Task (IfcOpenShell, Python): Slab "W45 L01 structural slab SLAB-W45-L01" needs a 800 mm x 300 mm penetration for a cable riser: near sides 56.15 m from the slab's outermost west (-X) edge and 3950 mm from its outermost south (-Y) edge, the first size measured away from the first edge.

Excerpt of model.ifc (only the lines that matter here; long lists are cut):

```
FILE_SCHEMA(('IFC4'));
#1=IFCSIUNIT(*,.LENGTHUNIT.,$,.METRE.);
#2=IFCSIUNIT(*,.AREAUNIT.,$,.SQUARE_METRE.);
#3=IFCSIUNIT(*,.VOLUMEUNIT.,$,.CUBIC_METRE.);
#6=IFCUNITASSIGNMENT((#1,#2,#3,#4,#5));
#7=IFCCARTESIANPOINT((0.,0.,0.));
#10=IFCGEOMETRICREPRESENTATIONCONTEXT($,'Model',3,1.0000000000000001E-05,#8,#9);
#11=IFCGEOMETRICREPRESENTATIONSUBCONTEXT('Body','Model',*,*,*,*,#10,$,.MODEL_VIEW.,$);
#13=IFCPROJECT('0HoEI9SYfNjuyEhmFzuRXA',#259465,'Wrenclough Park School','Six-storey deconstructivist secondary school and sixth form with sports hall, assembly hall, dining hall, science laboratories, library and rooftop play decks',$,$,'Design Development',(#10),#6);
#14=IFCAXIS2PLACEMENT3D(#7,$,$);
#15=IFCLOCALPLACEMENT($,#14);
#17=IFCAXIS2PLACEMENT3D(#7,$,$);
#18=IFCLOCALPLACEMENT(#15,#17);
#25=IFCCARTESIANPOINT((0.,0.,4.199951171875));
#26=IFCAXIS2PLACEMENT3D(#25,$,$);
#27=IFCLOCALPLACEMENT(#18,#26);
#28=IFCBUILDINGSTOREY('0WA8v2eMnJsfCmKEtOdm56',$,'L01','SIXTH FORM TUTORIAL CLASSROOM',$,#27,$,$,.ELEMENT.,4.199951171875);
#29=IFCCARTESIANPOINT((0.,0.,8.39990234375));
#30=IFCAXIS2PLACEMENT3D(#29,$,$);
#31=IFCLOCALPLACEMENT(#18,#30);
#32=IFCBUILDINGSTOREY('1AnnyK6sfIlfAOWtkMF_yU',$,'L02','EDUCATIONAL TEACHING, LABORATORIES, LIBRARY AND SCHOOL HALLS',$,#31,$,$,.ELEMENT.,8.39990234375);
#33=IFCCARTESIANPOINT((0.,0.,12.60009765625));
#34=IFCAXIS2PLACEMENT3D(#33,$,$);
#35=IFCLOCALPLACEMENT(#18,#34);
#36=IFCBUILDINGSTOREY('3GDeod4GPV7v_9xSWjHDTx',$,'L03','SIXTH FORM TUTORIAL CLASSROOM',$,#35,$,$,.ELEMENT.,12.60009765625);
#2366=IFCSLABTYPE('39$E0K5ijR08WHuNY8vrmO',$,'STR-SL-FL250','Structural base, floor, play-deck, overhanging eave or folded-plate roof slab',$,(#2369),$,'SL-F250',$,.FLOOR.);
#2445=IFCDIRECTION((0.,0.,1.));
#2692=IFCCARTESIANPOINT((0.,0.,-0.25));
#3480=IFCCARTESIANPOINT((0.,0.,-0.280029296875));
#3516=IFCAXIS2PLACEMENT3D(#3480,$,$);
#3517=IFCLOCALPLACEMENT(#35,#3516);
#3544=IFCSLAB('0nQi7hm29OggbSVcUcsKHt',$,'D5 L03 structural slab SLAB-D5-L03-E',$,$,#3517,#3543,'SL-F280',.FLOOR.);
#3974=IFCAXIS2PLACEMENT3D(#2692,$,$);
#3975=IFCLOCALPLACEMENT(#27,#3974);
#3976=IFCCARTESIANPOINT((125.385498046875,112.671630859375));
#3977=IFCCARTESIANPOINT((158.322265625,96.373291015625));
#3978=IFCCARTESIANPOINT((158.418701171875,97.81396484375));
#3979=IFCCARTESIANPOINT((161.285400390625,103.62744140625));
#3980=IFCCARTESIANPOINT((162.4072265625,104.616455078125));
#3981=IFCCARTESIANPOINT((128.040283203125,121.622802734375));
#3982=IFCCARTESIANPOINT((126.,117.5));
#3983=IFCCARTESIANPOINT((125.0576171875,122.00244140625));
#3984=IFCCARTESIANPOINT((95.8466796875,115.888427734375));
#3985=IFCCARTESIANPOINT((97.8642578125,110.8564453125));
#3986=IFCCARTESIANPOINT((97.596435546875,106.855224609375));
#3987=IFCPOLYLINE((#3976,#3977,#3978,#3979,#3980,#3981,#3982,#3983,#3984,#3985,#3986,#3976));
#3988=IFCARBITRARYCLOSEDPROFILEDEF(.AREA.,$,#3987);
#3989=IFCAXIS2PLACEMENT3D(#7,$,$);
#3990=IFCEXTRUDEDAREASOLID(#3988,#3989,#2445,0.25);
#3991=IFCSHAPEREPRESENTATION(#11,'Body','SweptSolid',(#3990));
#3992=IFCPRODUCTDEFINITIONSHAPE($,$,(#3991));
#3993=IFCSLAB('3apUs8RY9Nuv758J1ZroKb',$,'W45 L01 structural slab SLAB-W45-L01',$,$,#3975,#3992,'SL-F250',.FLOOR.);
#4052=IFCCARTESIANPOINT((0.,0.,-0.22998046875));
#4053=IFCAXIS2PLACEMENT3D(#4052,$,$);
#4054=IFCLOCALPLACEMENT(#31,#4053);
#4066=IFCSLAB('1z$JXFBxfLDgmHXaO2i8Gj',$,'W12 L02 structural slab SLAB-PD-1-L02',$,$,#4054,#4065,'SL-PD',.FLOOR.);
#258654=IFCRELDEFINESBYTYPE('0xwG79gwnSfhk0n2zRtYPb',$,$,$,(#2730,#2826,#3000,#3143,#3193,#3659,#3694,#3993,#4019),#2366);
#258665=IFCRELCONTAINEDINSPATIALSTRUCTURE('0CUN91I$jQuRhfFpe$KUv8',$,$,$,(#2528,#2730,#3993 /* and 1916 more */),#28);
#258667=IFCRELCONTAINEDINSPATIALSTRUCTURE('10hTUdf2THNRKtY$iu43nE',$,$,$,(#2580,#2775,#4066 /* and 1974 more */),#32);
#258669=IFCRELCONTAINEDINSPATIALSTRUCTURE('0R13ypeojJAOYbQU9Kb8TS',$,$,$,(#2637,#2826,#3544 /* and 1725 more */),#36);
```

```python
import numpy as np
import ifcopenshell
import ifcopenshell.api.feature
import ifcopenshell.api.geometry
import ifcopenshell.api.root
import ifcopenshell.geom
import ifcopenshell.util.placement
import ifcopenshell.util.representation
import ifcopenshell.util.shape
import ifcopenshell.util.unit

model = ifcopenshell.open("model.ifc")
unit_scale = ifcopenshell.util.unit.calculate_unit_scale(model)
settings = ifcopenshell.geom.settings()


def volume(element):
    """Net volume in cubic metres, openings subtracted."""
    shape = ifcopenshell.geom.create_shape(settings, element)
    return ifcopenshell.util.shape.get_volume(shape.geometry)


slab = model.by_guid("3apUs8RY9Nuv758J1ZroKb")
before = volume(slab)

# Extent in the slab's own axes, in metres. The edges named are its -X and -Y sides.
slab_shape = ifcopenshell.geom.create_shape(settings, slab)
vertices = ifcopenshell.util.shape.get_vertices(slab_shape.geometry)
x_min, y_min, bottom = vertices.min(axis=0)
top = vertices[:, 2].max()

opening = ifcopenshell.api.root.create_entity(model, ifc_class="IfcOpeningElement", name="Cable riser opening", predefined_type="OPENING")
context = ifcopenshell.util.representation.get_context(model, "Model", "Body", "MODEL_VIEW")
width, depth = 0.8, 0.3
outline = [(0.0, 0.0), (width, 0.0), (width, depth), (0.0, depth), (0.0, 0.0)]
# Overshoot both faces by 50 mm so the cut is clean.
shape = ifcopenshell.api.geometry.add_slab_representation(
    model, context=context, depth=top - bottom + 0.1, polyline=outline
)
ifcopenshell.api.geometry.assign_representation(model, product=opening, representation=shape)

matrix = ifcopenshell.util.placement.get_local_placement(slab.ObjectPlacement)
matrix[:, 3] = matrix @ np.append(np.array([x_min + 56.15, y_min + 3.95, bottom - 0.05]) / unit_scale, 1.0)
ifcopenshell.api.geometry.edit_object_placement(model, product=opening, matrix=matrix, is_si=False)
ifcopenshell.api.feature.add_feature(model, feature=opening, element=slab)

after = volume(slab)

print(f"slab volume {before:.3f} -> {after:.3f} m3")

model.write("model-out.ifc")
```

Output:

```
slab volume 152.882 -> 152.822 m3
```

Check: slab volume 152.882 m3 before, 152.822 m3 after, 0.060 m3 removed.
